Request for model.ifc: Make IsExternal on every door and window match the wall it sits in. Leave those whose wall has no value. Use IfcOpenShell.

First a look at what the model holds.

```python
import ifcopenshell
import ifcopenshell.util.element

model = ifcopenshell.open("model.ifc")
print(model.schema)
seen = {}
for e in model.by_type("IfcDoor") + model.by_type("IfcWindow"):
    if not e.FillsVoids:
        continue
    host = e.FillsVoids[0].RelatingOpeningElement.VoidsElements[0].RelatingBuildingElement
    own = ifcopenshell.util.element.get_pset(e, f"Pset_{e.is_a()[3:].removesuffix('StandardCase')}Common", "IsExternal")
    wall = ifcopenshell.util.element.get_pset(host, "Pset_WallCommon", "IsExternal")
    seen[e.is_a(), own, wall] = seen.get((e.is_a(), own, wall), 0) + 1
for (cls, own, wall), count in sorted(seen.items(), key=str):
    print(count, cls, "IsExternal:", own, "| host wall:", wall)
```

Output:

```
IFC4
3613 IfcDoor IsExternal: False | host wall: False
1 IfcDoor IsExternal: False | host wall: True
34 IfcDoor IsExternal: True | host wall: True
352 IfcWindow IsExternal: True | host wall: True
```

```python
import ifcopenshell
import ifcopenshell.api.pset
import ifcopenshell.util.element

model = ifcopenshell.open("model.ifc")

count = 0
for ifc_class, pset_name in (("IfcDoor", "Pset_DoorCommon"), ("IfcWindow", "Pset_WindowCommon")):
    for e in model.by_type(ifc_class):
        if not e.FillsVoids:
            continue
        host = e.FillsVoids[0].RelatingOpeningElement.VoidsElements[0].RelatingBuildingElement
        external = ifcopenshell.util.element.get_pset(host, "Pset_WallCommon", "IsExternal")
        if external is None or ifcopenshell.util.element.get_pset(e, pset_name, "IsExternal") == external:
            continue
        pset = ifcopenshell.api.pset.add_pset(model, product=e, name=pset_name)
        ifcopenshell.api.pset.edit_pset(model, pset=pset, properties={"IsExternal": external})
        count += 1

print(count, "updated")

model.write("model_rev.ifc")
```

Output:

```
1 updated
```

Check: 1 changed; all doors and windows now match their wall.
